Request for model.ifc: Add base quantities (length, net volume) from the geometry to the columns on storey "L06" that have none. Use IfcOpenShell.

First a look at what the model holds.

```python
import ifcopenshell
import ifcopenshell.util.element
import ifcopenshell.util.unit

model = ifcopenshell.open("model.ifc")
print(model.schema)
for unit_type in ("LENGTHUNIT", "AREAUNIT", "VOLUMEUNIT"):
    print(unit_type, ifcopenshell.util.unit.calculate_unit_scale(model, unit_type))
storey = next(s for s in model.by_type("IfcBuildingStorey") if s.Name == "L06")
columns = [e for e in ifcopenshell.util.element.get_decomposition(storey) if e.is_a("IfcColumn")]
for e in sorted(columns, key=lambda e: e.id()):
    print(e.id(), e.is_a(), e.Name, list(ifcopenshell.util.element.get_psets(e, qtos_only=True)), sep=" | ")
```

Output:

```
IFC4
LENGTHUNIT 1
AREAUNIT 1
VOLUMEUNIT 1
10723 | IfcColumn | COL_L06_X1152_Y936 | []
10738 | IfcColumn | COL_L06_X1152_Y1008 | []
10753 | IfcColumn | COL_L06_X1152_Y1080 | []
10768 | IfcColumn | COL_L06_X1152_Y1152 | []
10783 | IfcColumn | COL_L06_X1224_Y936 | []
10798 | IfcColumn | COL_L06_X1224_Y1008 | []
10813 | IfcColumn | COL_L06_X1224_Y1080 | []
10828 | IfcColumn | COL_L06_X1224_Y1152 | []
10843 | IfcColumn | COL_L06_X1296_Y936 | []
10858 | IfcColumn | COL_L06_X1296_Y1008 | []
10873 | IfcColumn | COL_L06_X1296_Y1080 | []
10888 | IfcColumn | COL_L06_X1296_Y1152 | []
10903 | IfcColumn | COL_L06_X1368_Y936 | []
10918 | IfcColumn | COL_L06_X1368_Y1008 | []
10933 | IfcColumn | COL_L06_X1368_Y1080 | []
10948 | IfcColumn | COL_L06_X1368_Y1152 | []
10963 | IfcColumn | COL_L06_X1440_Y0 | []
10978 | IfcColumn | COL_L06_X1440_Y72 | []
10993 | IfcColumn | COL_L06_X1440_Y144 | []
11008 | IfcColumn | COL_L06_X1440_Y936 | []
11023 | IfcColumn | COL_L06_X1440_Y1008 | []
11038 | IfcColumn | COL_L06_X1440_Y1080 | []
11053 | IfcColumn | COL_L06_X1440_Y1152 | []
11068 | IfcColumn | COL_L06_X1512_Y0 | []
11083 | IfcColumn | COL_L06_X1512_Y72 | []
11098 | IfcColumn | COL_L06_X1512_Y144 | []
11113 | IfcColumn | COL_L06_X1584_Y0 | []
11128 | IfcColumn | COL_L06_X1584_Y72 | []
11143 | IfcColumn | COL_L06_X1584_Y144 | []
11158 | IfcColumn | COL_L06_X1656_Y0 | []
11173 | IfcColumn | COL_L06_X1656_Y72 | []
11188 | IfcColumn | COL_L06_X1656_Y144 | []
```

```python
import ifcopenshell
import ifcopenshell.api.pset
import ifcopenshell.geom
import ifcopenshell.util.element
import ifcopenshell.util.shape
import ifcopenshell.util.unit

model = ifcopenshell.open("model.ifc")
unit_scale = ifcopenshell.util.unit.calculate_unit_scale(model)
volume_scale = ifcopenshell.util.unit.calculate_unit_scale(model, "VOLUMEUNIT")
settings = ifcopenshell.geom.settings()

storey = next(s for s in model.by_type("IfcBuildingStorey") if s.Name == "L06")
columns = [e for e in ifcopenshell.util.element.get_decomposition(storey) if e.is_a("IfcColumn")]

for e in sorted(columns, key=lambda e: e.id()):
    if ifcopenshell.util.element.get_psets(e, qtos_only=True, should_inherit=False):
        continue
    # Geometry comes back in metres, in the element's own axes.
    shape = ifcopenshell.geom.create_shape(settings, e)
    values = {
        "Length": ifcopenshell.util.shape.get_z(shape.geometry) / unit_scale,
        "NetVolume": ifcopenshell.util.shape.get_volume(shape.geometry) / volume_scale,
    }
    qto = ifcopenshell.api.pset.add_qto(model, product=e, name="Qto_ColumnBaseQuantities")
    ifcopenshell.api.pset.edit_qto(model, qto=qto, properties=values)
    print(e.id(), {k: round(v, 3) for k, v in values.items()})

model.write("model_updated.ifc")
```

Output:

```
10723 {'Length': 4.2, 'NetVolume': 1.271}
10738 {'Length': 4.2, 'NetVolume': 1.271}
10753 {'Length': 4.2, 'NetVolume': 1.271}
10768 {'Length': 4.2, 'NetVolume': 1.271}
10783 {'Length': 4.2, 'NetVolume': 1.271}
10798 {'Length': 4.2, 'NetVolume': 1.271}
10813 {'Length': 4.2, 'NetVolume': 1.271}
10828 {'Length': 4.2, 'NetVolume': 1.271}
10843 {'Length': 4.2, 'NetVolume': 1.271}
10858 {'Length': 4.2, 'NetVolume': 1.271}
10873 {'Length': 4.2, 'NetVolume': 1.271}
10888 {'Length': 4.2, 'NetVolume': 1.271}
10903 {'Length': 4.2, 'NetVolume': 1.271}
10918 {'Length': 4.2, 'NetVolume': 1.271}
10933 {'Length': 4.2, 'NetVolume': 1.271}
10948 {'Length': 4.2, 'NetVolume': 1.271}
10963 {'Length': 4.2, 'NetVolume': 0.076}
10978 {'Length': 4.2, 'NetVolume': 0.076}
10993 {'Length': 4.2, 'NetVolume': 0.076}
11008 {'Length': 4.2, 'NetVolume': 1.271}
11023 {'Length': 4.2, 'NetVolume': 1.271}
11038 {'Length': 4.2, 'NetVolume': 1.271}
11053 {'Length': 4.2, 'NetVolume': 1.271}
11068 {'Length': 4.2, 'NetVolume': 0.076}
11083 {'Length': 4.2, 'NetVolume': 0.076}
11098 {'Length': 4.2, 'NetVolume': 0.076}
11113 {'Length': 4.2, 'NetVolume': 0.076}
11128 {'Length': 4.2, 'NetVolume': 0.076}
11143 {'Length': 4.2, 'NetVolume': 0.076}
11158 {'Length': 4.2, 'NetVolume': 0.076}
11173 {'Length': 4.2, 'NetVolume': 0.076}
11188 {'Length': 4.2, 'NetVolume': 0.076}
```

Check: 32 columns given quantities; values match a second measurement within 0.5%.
